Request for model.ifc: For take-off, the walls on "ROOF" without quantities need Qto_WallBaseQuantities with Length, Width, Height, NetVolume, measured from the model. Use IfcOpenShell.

First a look at what the model holds.

```python
import ifcopenshell
import ifcopenshell.util.element
import ifcopenshell.util.unit

model = ifcopenshell.open("model.ifc")
print(model.schema)
for unit_type in ("LENGTHUNIT", "AREAUNIT", "VOLUMEUNIT"):
    print(unit_type, ifcopenshell.util.unit.calculate_unit_scale(model, unit_type))
storey = next(s for s in model.by_type("IfcBuildingStorey") if s.Name == "ROOF")
walls = [e for e in ifcopenshell.util.element.get_decomposition(storey) if e.is_a("IfcWall")]
for e in sorted(walls, key=lambda e: e.id()):
    print(e.id(), e.is_a(), e.Name, list(ifcopenshell.util.element.get_psets(e, qtos_only=True)), sep=" | ")
```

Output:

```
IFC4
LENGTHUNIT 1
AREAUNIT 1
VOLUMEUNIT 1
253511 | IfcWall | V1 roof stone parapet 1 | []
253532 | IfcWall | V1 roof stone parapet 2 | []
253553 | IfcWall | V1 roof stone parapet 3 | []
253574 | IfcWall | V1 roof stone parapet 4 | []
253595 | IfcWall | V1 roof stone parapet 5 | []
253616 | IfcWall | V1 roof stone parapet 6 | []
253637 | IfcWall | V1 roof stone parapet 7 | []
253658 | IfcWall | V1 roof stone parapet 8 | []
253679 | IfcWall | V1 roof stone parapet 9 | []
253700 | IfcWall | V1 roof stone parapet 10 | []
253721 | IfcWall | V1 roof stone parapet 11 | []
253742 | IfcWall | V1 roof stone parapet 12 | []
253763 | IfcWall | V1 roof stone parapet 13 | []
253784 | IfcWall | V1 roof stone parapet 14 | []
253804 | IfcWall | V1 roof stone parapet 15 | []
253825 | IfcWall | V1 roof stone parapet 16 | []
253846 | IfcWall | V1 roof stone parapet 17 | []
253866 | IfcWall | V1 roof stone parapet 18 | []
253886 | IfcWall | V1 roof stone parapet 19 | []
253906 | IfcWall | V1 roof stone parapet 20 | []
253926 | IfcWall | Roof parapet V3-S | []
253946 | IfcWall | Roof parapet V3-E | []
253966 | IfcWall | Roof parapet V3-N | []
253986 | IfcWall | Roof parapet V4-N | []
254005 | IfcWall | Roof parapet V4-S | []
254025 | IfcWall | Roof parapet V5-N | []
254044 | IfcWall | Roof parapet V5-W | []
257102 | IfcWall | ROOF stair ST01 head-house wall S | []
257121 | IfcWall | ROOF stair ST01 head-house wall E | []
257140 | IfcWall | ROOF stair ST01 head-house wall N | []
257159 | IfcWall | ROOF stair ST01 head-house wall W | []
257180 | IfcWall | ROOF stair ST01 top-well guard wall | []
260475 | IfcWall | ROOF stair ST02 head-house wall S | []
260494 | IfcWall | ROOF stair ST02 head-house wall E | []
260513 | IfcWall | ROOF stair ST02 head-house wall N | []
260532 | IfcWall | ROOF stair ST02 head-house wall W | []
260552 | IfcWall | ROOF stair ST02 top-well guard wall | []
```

```python
import ifcopenshell
import ifcopenshell.api.pset
import ifcopenshell.geom
import ifcopenshell.util.element
import ifcopenshell.util.shape
import ifcopenshell.util.unit

model = ifcopenshell.open("model.ifc")
unit_scale = ifcopenshell.util.unit.calculate_unit_scale(model)
volume_scale = ifcopenshell.util.unit.calculate_unit_scale(model, "VOLUMEUNIT")
settings = ifcopenshell.geom.settings()

storey = next(s for s in model.by_type("IfcBuildingStorey") if s.Name == "ROOF")
walls = [e for e in ifcopenshell.util.element.get_decomposition(storey) if e.is_a("IfcWall")]

for e in sorted(walls, key=lambda e: e.id()):
    if ifcopenshell.util.element.get_psets(e, qtos_only=True, should_inherit=False):
        continue
    # Geometry comes back in metres, in the element's own axes.
    shape = ifcopenshell.geom.create_shape(settings, e)
    values = {
        "Length": ifcopenshell.util.shape.get_x(shape.geometry) / unit_scale,
        "Width": ifcopenshell.util.shape.get_y(shape.geometry) / unit_scale,
        "Height": ifcopenshell.util.shape.get_z(shape.geometry) / unit_scale,
        "NetVolume": ifcopenshell.util.shape.get_volume(shape.geometry) / volume_scale,
    }
    qto = ifcopenshell.api.pset.add_qto(model, product=e, name="Qto_WallBaseQuantities")
    ifcopenshell.api.pset.edit_qto(model, qto=qto, properties=values)
    print(e.id(), {k: round(v, 3) for k, v in values.items()})

model.write("model_edited.ifc")
```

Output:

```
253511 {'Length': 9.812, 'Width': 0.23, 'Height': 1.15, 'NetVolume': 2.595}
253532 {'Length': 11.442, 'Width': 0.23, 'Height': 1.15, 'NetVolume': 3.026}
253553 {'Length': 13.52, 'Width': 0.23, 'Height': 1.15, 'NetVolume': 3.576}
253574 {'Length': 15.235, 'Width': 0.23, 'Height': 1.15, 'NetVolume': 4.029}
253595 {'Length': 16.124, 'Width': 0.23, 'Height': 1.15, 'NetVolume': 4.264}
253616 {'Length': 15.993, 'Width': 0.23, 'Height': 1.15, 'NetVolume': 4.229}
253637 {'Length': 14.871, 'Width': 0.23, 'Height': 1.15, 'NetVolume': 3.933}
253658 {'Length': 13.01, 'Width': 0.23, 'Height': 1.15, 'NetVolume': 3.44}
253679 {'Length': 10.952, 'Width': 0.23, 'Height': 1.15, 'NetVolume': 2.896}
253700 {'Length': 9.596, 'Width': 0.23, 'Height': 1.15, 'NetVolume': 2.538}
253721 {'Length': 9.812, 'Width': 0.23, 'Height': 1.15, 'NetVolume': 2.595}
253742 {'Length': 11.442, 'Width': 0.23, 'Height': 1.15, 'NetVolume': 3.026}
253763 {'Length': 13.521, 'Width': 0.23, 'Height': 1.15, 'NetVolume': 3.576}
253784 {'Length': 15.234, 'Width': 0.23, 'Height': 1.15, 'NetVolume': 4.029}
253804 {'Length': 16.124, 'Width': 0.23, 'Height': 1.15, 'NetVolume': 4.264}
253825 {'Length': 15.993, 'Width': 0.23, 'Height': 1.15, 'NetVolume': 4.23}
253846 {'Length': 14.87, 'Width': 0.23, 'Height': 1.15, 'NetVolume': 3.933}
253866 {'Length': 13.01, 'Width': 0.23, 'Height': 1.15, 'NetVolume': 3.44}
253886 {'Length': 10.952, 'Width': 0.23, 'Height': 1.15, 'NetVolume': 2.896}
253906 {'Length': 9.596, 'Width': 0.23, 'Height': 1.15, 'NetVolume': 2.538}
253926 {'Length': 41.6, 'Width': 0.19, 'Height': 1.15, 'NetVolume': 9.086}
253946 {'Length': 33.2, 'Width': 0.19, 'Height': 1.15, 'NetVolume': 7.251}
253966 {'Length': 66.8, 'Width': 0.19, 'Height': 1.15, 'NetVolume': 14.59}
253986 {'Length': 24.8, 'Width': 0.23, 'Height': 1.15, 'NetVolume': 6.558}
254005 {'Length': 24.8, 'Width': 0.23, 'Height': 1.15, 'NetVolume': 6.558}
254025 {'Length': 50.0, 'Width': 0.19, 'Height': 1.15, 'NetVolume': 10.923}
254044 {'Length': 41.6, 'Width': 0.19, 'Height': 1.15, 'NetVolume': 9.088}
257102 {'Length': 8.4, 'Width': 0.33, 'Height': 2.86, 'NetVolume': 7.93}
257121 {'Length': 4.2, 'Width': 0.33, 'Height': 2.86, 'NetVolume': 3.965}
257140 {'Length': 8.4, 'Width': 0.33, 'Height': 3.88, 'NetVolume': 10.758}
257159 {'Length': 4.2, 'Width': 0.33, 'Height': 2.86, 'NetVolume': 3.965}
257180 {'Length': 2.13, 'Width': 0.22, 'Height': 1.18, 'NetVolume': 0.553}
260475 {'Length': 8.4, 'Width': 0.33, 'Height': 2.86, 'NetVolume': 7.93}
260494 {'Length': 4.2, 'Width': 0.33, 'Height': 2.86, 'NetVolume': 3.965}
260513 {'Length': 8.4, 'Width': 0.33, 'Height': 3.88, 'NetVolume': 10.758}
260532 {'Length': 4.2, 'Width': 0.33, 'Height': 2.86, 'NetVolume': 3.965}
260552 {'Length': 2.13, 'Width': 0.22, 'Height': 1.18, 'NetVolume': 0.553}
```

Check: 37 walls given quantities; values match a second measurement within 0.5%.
